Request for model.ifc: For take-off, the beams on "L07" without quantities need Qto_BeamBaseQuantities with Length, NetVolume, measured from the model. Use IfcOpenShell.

First a look at what the model holds.

```python
import ifcopenshell
import ifcopenshell.util.element
import ifcopenshell.util.unit

model = ifcopenshell.open("model.ifc")
print(model.schema)
for unit_type in ("LENGTHUNIT", "AREAUNIT", "VOLUMEUNIT"):
    print(unit_type, ifcopenshell.util.unit.calculate_unit_scale(model, unit_type))
storey = next(s for s in model.by_type("IfcBuildingStorey") if s.Name == "L07")
beams = [e for e in ifcopenshell.util.element.get_decomposition(storey) if e.is_a("IfcBeam")]
for e in sorted(beams, key=lambda e: e.id()):
    print(e.id(), e.is_a(), e.Name, list(ifcopenshell.util.element.get_psets(e, qtos_only=True)), sep=" | ")
```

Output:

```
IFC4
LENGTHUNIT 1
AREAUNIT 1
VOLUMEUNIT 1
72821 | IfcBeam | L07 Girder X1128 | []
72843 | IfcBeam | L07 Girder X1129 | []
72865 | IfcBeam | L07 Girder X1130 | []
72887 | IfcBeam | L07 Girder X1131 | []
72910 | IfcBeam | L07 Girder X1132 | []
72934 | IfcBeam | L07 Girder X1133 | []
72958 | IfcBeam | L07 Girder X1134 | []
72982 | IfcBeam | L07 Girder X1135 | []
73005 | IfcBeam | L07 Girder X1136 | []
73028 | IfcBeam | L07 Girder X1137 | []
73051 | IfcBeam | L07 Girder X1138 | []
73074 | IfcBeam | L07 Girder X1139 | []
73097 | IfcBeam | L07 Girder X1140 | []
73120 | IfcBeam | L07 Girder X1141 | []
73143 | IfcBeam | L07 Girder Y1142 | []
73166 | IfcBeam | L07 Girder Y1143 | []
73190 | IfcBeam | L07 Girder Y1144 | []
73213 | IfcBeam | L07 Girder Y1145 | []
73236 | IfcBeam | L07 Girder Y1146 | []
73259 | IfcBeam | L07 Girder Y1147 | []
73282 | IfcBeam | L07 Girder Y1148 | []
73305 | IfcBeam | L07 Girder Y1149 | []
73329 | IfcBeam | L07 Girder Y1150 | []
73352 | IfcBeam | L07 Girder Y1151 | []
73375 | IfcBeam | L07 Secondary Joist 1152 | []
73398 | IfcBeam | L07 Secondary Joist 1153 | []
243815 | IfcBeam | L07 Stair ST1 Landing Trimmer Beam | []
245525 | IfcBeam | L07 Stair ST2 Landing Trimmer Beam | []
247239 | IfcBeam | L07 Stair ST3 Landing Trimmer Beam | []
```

```python
import ifcopenshell
import ifcopenshell.api.pset
import ifcopenshell.geom
import ifcopenshell.util.element
import ifcopenshell.util.shape
import ifcopenshell.util.unit

model = ifcopenshell.open("model.ifc")
unit_scale = ifcopenshell.util.unit.calculate_unit_scale(model)
volume_scale = ifcopenshell.util.unit.calculate_unit_scale(model, "VOLUMEUNIT")
settings = ifcopenshell.geom.settings()

storey = next(s for s in model.by_type("IfcBuildingStorey") if s.Name == "L07")
beams = [e for e in ifcopenshell.util.element.get_decomposition(storey) if e.is_a("IfcBeam")]

for e in sorted(beams, key=lambda e: e.id()):
    if ifcopenshell.util.element.get_psets(e, qtos_only=True, should_inherit=False):
        continue
    # Geometry comes back in metres, in the element's own axes.
    shape = ifcopenshell.geom.create_shape(settings, e)
    values = {
        "Length": ifcopenshell.util.shape.get_max_xyz(shape.geometry) / unit_scale,
        "NetVolume": ifcopenshell.util.shape.get_volume(shape.geometry) / volume_scale,
    }
    qto = ifcopenshell.api.pset.add_qto(model, product=e, name="Qto_BeamBaseQuantities")
    ifcopenshell.api.pset.edit_qto(model, qto=qto, properties=values)
    print(e.id(), {k: round(v, 3) for k, v in values.items()})

model.write("model-out.ifc")
```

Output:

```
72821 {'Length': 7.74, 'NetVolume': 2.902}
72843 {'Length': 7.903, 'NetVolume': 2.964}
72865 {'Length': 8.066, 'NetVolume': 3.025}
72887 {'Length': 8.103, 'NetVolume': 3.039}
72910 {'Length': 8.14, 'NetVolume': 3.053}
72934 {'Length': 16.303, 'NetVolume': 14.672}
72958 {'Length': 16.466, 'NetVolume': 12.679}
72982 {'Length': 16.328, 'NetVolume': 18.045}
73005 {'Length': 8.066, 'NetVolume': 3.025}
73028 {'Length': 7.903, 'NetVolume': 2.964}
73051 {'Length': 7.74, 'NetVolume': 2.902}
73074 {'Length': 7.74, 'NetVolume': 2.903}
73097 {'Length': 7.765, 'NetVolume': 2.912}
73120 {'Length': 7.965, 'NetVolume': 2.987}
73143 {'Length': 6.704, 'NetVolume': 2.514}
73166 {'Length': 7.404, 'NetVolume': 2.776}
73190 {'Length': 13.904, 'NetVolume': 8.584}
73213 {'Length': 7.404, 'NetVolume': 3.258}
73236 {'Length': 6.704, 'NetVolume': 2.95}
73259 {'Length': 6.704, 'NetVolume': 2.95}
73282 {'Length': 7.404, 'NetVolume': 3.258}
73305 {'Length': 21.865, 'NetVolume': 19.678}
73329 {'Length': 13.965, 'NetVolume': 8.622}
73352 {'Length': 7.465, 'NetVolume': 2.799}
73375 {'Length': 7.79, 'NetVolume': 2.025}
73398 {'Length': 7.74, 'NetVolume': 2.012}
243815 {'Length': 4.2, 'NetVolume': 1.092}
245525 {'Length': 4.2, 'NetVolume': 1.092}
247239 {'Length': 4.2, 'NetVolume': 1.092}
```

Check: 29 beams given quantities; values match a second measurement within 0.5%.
